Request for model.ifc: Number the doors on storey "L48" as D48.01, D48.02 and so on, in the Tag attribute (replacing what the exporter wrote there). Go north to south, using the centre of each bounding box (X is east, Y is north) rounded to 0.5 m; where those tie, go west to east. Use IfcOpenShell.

First a look at what the model holds.

```python
import ifcopenshell
import ifcopenshell.util.element
import ifcopenshell.util.placement

model = ifcopenshell.open("model.ifc")
print(model.schema)
storey = next(s for s in model.by_type("IfcBuildingStorey") if s.Name == "L48")
doors = [e for e in ifcopenshell.util.element.get_decomposition(storey) if e.is_a("IfcDoor")]
for e in sorted(doors, key=lambda e: e.id()):
    origin = ifcopenshell.util.placement.get_local_placement(e.ObjectPlacement)[:3, 3]
    print(e.id(), e.Tag, e.Name, origin.round(2) + 0.0, sep=" | ")
```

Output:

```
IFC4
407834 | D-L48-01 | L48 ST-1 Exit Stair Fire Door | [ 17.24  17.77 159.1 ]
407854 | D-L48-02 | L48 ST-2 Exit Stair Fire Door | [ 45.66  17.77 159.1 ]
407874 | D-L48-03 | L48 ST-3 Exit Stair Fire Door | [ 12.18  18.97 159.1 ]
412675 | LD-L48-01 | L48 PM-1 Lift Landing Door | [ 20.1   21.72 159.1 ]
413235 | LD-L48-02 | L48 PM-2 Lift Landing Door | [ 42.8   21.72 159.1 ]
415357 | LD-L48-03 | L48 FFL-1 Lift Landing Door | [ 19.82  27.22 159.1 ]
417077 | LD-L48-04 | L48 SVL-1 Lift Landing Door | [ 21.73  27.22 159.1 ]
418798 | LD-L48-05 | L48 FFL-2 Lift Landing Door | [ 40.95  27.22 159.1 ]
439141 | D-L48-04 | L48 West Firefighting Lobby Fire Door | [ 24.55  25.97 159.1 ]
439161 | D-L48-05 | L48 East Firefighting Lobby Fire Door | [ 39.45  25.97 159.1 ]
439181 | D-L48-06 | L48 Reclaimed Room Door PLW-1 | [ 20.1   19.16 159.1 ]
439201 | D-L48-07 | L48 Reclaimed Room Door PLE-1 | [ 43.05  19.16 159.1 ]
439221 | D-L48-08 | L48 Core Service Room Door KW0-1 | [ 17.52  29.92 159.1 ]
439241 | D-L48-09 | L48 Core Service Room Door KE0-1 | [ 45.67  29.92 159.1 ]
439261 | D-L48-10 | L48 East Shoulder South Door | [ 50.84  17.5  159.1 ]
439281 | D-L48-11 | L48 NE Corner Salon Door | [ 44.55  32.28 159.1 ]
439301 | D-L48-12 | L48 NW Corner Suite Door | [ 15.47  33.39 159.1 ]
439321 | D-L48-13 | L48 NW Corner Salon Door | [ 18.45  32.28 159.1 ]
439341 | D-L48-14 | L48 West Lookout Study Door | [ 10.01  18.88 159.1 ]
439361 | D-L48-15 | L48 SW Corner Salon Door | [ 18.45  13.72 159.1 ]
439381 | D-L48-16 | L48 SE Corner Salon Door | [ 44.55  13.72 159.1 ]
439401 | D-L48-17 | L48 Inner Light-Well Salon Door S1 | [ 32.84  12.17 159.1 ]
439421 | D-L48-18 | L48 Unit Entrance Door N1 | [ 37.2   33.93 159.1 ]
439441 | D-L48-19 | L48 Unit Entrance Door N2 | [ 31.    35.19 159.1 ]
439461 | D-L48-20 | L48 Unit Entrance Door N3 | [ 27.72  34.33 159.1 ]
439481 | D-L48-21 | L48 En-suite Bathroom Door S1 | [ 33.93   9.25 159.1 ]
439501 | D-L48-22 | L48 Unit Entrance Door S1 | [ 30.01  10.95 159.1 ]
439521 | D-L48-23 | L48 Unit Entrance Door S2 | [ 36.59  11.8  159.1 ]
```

```python
import ifcopenshell
import ifcopenshell.geom
import ifcopenshell.util.element
import ifcopenshell.util.shape

model = ifcopenshell.open("model.ifc")
settings = ifcopenshell.geom.settings()
settings.set("use-world-coords", True)


def centre(element):
    shape = ifcopenshell.geom.create_shape(settings, element)
    return ifcopenshell.util.shape.get_bbox_centroid(shape.geometry)


storey = next(s for s in model.by_type("IfcBuildingStorey") if s.Name == "L48")
doors = [e for e in ifcopenshell.util.element.get_decomposition(storey) if e.is_a("IfcDoor")]

# Insertion points can sit at a corner or the storey origin, so sort by the geometry (in metres).
centres = {e: centre(e) for e in doors}
doors.sort(key=lambda e: (-round(centres[e][1] / 0.5), centres[e][0]))

for i, e in enumerate(doors, start=1):
    number = f"D48.{i:02d}"
    e.Tag = number
    print(e.id(), number)

model.write("model_updated.ifc")
```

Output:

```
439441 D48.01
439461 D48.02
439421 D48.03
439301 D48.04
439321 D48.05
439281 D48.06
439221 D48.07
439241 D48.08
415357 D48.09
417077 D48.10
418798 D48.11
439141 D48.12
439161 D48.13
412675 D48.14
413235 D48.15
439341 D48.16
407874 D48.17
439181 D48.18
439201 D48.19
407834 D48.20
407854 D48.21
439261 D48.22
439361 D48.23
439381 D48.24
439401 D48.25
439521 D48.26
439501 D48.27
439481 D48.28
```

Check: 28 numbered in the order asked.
